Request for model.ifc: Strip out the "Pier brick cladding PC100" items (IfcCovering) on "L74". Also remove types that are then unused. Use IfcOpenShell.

First a look at what the model holds.

```python
import ifcopenshell
import ifcopenshell.util.element

model = ifcopenshell.open("model.ifc")
print(model.schema)
storey = next(s for s in model.by_type("IfcBuildingStorey") if s.Name == "L74")
coverings = [e for e in ifcopenshell.util.element.get_decomposition(storey) if e.is_a("IfcCovering")]
seen = {}
for e in coverings:
    element_type = ifcopenshell.util.element.get_type(e)
    name = element_type.Name if element_type not in (None, e) else None
    seen[name] = seen.get(name, 0) + 1
for name, count in sorted(seen.items(), key=str):
    print(count, "x", name)
```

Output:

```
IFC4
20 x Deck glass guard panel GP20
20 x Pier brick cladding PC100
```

```python
import ifcopenshell
import ifcopenshell.api.root
import ifcopenshell.util.element

model = ifcopenshell.open("model.ifc")

storey = next(s for s in model.by_type("IfcBuildingStorey") if s.Name == "L74")
coverings = [e for e in ifcopenshell.util.element.get_decomposition(storey) if e.is_a("IfcCovering")]
targets = [e for e in coverings if (t := ifcopenshell.util.element.get_type(e)) not in (None, e) and t.Name == "Pier brick cladding PC100"]
types = {ifcopenshell.util.element.get_type(e) for e in targets} - {None, *targets}

for e in targets:
    ifcopenshell.api.root.remove_product(model, product=e)
print(len(targets), "removed")

unused = [t for t in types if not ifcopenshell.util.element.get_types(t)]
for t in unused:
    ifcopenshell.api.root.remove_product(model, product=t)
print(len(unused), "unused types removed")

model.write("model_edited.ifc")
```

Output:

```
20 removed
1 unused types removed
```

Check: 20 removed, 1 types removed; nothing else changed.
